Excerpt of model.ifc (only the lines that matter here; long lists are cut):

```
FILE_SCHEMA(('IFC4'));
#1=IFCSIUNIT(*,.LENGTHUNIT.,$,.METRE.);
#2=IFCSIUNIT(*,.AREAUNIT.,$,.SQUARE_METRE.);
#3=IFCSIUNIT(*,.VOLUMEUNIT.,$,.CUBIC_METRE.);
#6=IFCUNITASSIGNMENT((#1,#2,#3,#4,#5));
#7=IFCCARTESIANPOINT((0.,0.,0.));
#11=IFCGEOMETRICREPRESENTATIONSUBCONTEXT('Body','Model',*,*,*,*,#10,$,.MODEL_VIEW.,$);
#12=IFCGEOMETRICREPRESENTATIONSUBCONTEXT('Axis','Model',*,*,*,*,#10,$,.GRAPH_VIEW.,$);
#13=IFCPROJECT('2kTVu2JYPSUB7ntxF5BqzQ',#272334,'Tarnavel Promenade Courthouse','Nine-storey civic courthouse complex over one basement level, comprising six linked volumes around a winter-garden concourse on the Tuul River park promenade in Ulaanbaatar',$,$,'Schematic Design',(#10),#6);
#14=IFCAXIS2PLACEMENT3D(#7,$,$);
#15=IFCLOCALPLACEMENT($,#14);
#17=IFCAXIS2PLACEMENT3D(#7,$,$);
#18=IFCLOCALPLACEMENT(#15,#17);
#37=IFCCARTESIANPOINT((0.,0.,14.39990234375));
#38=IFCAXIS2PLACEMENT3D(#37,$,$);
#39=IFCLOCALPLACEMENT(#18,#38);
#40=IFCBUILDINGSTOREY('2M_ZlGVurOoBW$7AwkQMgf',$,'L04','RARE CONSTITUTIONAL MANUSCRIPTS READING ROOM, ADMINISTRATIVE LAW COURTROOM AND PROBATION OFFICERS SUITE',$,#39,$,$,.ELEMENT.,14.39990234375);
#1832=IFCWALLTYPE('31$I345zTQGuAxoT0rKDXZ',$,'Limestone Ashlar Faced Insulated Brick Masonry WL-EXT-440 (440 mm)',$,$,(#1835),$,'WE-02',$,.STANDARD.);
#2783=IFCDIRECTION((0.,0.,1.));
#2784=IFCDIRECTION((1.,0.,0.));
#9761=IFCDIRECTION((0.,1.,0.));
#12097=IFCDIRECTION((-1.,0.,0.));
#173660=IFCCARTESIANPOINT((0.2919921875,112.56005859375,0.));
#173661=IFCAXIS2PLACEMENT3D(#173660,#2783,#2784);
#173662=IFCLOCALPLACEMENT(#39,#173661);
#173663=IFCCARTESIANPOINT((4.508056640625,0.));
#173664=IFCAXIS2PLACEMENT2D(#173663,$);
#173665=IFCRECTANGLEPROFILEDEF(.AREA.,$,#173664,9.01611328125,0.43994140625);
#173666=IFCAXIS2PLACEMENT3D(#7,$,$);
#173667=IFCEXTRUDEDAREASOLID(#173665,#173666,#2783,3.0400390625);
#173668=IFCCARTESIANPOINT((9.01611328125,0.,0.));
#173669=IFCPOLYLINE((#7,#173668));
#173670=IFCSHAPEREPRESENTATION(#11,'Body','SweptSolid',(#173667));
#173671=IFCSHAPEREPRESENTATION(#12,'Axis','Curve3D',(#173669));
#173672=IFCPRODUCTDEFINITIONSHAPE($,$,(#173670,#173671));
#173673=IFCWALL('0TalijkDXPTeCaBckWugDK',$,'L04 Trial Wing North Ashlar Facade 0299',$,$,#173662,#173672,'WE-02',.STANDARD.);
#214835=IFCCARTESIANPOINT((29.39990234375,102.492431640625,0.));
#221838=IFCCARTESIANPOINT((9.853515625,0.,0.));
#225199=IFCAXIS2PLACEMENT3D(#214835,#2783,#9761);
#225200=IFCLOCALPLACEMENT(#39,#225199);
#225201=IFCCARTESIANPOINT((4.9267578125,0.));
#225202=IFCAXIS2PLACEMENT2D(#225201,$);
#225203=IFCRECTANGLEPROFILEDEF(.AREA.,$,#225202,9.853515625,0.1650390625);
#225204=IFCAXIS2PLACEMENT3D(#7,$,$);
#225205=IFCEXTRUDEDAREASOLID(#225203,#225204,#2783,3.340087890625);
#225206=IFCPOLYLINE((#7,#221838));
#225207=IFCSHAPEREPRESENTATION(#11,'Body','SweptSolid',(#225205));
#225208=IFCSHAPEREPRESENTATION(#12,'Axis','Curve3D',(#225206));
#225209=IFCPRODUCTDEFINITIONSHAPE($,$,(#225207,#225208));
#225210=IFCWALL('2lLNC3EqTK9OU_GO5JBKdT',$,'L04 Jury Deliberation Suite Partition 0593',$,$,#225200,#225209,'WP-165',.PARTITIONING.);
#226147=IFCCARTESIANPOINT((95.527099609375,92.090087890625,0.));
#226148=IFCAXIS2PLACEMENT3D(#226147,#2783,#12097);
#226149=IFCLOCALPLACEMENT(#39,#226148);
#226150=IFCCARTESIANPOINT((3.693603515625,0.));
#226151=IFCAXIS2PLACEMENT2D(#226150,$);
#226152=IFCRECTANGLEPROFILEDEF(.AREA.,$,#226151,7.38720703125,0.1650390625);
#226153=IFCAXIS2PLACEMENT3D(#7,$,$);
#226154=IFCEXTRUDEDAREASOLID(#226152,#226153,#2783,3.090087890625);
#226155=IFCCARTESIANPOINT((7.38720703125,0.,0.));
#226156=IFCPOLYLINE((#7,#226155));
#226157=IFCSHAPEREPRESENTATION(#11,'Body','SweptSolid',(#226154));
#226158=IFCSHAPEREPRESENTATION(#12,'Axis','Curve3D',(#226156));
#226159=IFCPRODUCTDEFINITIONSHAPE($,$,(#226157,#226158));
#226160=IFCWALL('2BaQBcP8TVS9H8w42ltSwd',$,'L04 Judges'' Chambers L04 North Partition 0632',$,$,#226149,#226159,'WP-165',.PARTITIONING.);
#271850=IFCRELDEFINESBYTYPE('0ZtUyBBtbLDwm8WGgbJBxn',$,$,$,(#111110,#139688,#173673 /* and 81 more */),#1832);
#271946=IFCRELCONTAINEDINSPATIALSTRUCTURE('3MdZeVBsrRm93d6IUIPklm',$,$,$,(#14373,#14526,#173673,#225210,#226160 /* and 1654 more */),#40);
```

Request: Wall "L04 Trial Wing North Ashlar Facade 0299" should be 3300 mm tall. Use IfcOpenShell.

```python
import ifcopenshell
import ifcopenshell.geom
import ifcopenshell.util.representation
import ifcopenshell.util.shape
import ifcopenshell.util.unit

model = ifcopenshell.open("model.ifc")
unit_scale = ifcopenshell.util.unit.calculate_unit_scale(model)
settings = ifcopenshell.geom.settings()


def volume(element):
    """Net volume in cubic metres, openings subtracted."""
    shape = ifcopenshell.geom.create_shape(settings, element)
    return ifcopenshell.util.shape.get_volume(shape.geometry)


wall = model.by_id(173673)
before = volume(wall)

body = ifcopenshell.util.representation.get_representation(wall, "Model", "Body")
solid = body.Items[0]
old_height = solid.Depth
solid.Depth = 3.3 / unit_scale
after = volume(wall)

print(f"height {old_height:g} -> {solid.Depth:g}, volume {before:.3f} -> {after:.3f} m3")

model.write("model_edited.ifc")
```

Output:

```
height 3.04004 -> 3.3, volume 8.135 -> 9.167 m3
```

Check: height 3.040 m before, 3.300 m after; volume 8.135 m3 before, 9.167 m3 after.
